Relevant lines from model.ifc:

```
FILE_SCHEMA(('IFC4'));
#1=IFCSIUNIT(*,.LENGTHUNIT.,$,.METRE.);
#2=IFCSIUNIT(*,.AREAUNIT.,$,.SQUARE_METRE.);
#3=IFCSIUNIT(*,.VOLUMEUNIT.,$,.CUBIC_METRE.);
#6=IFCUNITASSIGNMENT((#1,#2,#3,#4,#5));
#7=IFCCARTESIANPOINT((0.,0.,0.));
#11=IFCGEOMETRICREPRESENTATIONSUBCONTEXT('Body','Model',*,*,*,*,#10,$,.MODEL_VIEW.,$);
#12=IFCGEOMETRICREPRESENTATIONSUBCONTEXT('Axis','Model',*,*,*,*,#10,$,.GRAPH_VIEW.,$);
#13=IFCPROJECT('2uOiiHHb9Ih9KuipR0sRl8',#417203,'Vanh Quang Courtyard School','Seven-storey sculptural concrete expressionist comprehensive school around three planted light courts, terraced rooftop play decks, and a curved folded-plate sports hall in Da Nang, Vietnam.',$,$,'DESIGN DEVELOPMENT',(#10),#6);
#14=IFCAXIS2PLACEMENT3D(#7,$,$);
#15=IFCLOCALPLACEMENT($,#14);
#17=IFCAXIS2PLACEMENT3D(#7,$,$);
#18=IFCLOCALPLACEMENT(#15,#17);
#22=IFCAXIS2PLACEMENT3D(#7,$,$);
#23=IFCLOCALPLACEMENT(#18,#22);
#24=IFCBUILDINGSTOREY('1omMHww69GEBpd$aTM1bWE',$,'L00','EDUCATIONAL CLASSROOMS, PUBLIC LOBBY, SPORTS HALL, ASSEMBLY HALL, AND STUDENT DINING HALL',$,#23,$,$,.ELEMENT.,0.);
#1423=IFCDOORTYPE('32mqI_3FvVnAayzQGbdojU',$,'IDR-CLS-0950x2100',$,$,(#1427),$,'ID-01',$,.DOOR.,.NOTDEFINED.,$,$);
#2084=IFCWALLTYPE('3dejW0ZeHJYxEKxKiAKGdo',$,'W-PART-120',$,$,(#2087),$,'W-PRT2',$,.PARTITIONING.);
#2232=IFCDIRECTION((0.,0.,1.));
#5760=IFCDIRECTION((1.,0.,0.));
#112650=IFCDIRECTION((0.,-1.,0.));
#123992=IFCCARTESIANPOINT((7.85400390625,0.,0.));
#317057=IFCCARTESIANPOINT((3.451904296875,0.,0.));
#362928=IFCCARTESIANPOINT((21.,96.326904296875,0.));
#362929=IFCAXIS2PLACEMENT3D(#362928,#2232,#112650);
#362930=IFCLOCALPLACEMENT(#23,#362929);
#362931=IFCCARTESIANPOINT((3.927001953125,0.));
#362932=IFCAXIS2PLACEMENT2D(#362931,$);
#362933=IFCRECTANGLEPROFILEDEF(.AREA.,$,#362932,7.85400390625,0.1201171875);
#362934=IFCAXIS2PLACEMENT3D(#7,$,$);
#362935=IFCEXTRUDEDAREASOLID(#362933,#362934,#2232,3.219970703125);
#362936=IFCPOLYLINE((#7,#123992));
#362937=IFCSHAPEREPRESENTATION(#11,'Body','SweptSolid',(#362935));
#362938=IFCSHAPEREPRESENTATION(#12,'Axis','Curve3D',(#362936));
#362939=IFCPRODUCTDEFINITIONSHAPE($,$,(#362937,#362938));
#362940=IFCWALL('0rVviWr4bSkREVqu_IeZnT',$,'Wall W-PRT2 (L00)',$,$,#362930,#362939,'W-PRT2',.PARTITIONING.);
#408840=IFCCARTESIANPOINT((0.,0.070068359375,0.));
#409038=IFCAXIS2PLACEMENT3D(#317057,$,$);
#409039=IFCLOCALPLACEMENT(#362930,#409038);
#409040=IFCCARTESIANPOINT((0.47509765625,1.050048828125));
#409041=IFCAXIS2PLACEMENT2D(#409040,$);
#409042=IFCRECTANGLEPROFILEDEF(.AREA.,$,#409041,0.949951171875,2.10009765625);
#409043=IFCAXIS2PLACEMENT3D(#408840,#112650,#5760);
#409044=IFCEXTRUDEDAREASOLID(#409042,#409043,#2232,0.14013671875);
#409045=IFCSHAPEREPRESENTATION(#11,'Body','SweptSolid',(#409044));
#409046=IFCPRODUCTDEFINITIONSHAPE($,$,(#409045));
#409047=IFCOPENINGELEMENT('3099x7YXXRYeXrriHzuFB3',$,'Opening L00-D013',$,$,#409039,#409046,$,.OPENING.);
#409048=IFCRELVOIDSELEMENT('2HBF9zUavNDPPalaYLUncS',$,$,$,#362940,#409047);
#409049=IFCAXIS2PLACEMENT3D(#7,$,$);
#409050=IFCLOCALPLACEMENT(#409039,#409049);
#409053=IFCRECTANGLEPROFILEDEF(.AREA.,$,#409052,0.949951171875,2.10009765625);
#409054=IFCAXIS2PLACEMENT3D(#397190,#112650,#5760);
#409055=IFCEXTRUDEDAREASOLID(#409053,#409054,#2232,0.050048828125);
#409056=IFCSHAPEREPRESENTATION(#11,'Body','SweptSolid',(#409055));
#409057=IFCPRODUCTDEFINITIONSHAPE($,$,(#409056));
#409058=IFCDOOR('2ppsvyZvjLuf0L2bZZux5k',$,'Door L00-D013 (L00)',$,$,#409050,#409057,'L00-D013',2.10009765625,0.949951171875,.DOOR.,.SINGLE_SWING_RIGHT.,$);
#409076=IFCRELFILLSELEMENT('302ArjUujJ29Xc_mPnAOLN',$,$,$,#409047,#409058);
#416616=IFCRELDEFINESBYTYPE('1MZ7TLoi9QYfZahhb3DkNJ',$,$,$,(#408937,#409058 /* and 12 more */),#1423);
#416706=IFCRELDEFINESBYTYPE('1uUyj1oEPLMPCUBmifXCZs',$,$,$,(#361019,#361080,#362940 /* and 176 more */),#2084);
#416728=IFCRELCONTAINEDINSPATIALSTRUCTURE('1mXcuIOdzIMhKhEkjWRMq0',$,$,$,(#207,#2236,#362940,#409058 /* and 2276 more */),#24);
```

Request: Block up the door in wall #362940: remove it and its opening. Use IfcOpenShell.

```python
import ifcopenshell
import ifcopenshell.api.feature
import ifcopenshell.api.root
import ifcopenshell.geom
import ifcopenshell.util.shape

model = ifcopenshell.open("model.ifc")
settings = ifcopenshell.geom.settings()


def volume(element):
    """Net volume in cubic metres, openings subtracted."""
    shape = ifcopenshell.geom.create_shape(settings, element)
    return ifcopenshell.util.shape.get_volume(shape.geometry)


door = model.by_guid("2ppsvyZvjLuf0L2bZZux5k")
opening = door.FillsVoids[0].RelatingOpeningElement
wall = opening.VoidsElements[0].RelatingBuildingElement
before = volume(wall)

ifcopenshell.api.root.remove_product(model, product=door)
ifcopenshell.api.feature.remove_feature(model, feature=opening)

after = volume(wall)

print(f"wall volume {before:.3f} -> {after:.3f} m3")

model.write("model_v2.ifc")
```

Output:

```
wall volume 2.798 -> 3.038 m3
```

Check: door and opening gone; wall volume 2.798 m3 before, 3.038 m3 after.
